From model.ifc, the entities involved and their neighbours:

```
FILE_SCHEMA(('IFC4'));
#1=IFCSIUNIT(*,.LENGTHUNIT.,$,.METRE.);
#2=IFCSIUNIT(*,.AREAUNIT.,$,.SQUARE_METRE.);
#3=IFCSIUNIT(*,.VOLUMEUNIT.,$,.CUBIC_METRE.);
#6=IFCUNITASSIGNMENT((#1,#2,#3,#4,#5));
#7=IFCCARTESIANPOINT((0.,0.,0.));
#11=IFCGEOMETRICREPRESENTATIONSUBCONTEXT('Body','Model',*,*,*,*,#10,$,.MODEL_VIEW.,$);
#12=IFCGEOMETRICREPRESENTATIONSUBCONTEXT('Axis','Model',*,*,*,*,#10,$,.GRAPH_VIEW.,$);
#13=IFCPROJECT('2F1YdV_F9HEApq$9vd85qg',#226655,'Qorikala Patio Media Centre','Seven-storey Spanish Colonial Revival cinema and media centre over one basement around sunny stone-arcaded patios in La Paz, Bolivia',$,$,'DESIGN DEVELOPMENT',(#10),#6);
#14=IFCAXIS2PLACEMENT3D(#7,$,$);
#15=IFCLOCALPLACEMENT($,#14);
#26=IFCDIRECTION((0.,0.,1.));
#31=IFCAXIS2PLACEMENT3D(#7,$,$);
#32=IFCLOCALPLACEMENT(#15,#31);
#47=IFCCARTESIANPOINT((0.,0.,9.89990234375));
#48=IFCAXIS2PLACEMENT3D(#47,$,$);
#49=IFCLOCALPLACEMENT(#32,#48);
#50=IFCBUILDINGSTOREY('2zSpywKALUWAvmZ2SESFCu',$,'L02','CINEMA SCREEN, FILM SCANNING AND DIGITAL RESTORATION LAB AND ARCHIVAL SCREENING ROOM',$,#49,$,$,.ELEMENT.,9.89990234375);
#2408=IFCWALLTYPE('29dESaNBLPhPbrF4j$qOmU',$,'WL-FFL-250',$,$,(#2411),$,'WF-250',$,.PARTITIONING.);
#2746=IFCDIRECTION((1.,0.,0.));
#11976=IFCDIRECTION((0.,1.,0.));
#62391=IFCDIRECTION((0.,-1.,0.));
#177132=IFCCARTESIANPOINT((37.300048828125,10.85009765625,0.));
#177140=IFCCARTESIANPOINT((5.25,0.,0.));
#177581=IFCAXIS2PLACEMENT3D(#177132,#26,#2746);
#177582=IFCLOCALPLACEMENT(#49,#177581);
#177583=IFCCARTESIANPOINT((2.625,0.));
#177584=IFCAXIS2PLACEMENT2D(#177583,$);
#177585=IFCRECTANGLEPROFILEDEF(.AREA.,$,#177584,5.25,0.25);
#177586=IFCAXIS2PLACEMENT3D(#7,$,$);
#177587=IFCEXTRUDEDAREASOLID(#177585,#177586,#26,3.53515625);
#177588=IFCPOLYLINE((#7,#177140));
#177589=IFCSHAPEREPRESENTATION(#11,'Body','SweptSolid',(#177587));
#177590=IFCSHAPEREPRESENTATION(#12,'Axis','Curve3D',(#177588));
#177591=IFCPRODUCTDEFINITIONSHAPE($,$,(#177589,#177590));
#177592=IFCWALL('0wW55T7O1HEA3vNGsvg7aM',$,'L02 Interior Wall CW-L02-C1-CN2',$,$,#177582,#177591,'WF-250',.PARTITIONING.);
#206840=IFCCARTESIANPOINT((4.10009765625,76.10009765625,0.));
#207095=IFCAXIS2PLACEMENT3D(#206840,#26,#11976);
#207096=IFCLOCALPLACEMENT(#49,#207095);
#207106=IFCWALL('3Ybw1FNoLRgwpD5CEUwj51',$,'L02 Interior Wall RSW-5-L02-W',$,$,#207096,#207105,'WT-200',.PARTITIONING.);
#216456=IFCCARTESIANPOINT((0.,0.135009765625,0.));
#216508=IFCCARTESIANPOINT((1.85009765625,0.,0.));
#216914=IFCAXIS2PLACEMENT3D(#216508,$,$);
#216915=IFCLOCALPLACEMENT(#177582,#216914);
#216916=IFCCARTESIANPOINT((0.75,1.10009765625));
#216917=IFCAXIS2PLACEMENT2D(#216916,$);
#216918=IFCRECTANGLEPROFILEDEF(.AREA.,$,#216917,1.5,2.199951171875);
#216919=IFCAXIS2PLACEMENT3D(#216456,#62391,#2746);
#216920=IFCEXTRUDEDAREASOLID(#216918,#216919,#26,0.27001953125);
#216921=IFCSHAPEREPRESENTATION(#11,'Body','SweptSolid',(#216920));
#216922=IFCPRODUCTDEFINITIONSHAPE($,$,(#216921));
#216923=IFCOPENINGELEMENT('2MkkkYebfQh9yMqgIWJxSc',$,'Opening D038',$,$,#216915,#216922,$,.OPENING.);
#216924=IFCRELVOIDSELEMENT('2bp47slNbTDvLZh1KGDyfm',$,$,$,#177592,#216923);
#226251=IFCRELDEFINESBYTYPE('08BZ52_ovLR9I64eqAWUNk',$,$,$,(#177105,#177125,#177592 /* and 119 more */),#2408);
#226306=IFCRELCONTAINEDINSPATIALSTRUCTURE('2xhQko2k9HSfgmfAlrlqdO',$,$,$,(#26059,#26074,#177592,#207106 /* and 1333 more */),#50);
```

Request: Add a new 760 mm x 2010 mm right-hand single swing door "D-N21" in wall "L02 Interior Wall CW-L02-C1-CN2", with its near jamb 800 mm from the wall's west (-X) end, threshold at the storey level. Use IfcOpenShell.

```python
import numpy as np
import ifcopenshell
import ifcopenshell.api.feature
import ifcopenshell.api.geometry
import ifcopenshell.api.root
import ifcopenshell.api.spatial
import ifcopenshell.geom
import ifcopenshell.util.element
import ifcopenshell.util.placement
import ifcopenshell.util.representation
import ifcopenshell.util.shape
import ifcopenshell.util.unit

model = ifcopenshell.open("model.ifc")
unit_scale = ifcopenshell.util.unit.calculate_unit_scale(model)
settings = ifcopenshell.geom.settings()


def volume(element):
    """Net volume in cubic metres, openings subtracted."""
    shape = ifcopenshell.geom.create_shape(settings, element)
    return ifcopenshell.util.shape.get_volume(shape.geometry)


wall = model.by_guid("0wW55T7O1HEA3vNGsvg7aM")
storey = ifcopenshell.util.element.get_container(wall, ifc_class="IfcBuildingStorey")
context = ifcopenshell.util.representation.get_context(model, "Model", "Body", "MODEL_VIEW")
before = volume(wall)

width, height, from_end, sill = 0.76, 2.01, 0.8, 0.0  # metres

# The wall runs along its own X axis, and the end named is its -X end.
wall_shape = ifcopenshell.geom.create_shape(settings, wall)
x, y, z = ifcopenshell.util.shape.get_vertices(wall_shape.geometry).T
start = x.min() + from_end
face, thickness = float(y.min()), float(y.max() - y.min())
wall_matrix = ifcopenshell.util.placement.get_local_placement(wall.ObjectPlacement)
level = ifcopenshell.util.placement.get_local_placement(storey.ObjectPlacement)[2, 3]


def in_wall(x, y):
    """Placement at x, y metres in the wall's axes, at sill height."""
    matrix = wall_matrix.copy()
    matrix[:, 3] = wall_matrix @ np.array([x / unit_scale, y / unit_scale, 0.0, 1.0])
    matrix[2, 3] = level + sill / unit_scale
    return matrix


# Opening: a box that overshoots both wall faces by 50 mm.
opening = ifcopenshell.api.root.create_entity(model, ifc_class="IfcOpeningElement", predefined_type="OPENING")
box = ifcopenshell.api.geometry.add_wall_representation(
    model, context=context, length=width, height=height, thickness=thickness + 0.1
)
ifcopenshell.api.geometry.assign_representation(model, product=opening, representation=box)
ifcopenshell.api.geometry.edit_object_placement(model, product=opening, matrix=in_wall(start, face - 0.05), is_si=False)
ifcopenshell.api.feature.add_feature(model, feature=opening, element=wall)

door = ifcopenshell.api.root.create_entity(model, ifc_class="IfcDoor", name="D-N21", predefined_type="DOOR")
door.OverallWidth, door.OverallHeight = width / unit_scale, height / unit_scale
door.OperationType = "SINGLE_SWING_RIGHT"
body = ifcopenshell.api.geometry.add_door_representation(
    model,
    context=context,
    overall_width=door.OverallWidth,
    overall_height=door.OverallHeight,
    operation_type="SINGLE_SWING_RIGHT",
    lining_properties={"LiningDepth": thickness / unit_scale, "ThresholdDepth": thickness / unit_scale},
)
ifcopenshell.api.geometry.assign_representation(model, product=door, representation=body)
ifcopenshell.api.spatial.assign_container(model, products=[door], relating_structure=storey)
ifcopenshell.api.feature.add_filling(model, opening=opening, element=door)

# The lining spans the wall, so the door starts at the wall face.
ifcopenshell.api.geometry.edit_object_placement(model, product=door, matrix=in_wall(start, face), is_si=False)

after = volume(wall)

print(f"wall volume {before:.3f} -> {after:.3f} m3")

model.write("model_edited.ifc")
```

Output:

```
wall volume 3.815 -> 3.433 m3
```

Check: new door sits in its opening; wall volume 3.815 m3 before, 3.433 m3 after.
